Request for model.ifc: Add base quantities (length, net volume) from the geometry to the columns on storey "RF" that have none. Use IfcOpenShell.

First a look at what the model holds.

```python
import ifcopenshell
import ifcopenshell.util.element
import ifcopenshell.util.unit

model = ifcopenshell.open("model.ifc")
print(model.schema)
for unit_type in ("LENGTHUNIT", "AREAUNIT", "VOLUMEUNIT"):
    print(unit_type, ifcopenshell.util.unit.calculate_unit_scale(model, unit_type))
storey = next(s for s in model.by_type("IfcBuildingStorey") if s.Name == "RF")
columns = [e for e in ifcopenshell.util.element.get_decomposition(storey) if e.is_a("IfcColumn")]
for e in sorted(columns, key=lambda e: e.id()):
    print(e.id(), e.is_a(), e.Name, list(ifcopenshell.util.element.get_psets(e, qtos_only=True)), sep=" | ")
```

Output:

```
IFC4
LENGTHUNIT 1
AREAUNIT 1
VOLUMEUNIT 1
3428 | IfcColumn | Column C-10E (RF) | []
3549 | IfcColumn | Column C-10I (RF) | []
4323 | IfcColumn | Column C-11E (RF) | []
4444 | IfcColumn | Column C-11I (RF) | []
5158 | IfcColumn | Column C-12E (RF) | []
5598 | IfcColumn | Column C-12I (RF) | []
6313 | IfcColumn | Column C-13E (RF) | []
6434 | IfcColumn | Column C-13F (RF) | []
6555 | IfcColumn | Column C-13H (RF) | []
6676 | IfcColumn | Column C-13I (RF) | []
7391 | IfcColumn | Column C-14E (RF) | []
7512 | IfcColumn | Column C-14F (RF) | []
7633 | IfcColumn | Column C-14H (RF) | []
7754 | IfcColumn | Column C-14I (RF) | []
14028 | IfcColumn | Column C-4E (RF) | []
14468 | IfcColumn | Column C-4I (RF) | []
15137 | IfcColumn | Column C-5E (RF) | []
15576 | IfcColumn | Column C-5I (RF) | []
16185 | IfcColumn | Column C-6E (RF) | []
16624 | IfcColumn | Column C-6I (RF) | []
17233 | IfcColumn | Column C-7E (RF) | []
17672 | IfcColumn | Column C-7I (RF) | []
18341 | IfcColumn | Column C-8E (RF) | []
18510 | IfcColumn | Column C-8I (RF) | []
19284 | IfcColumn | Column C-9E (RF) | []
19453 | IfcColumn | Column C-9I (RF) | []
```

```python
import ifcopenshell
import ifcopenshell.api.pset
import ifcopenshell.geom
import ifcopenshell.util.element
import ifcopenshell.util.shape
import ifcopenshell.util.unit

model = ifcopenshell.open("model.ifc")
unit_scale = ifcopenshell.util.unit.calculate_unit_scale(model)
volume_scale = ifcopenshell.util.unit.calculate_unit_scale(model, "VOLUMEUNIT")
settings = ifcopenshell.geom.settings()

storey = next(s for s in model.by_type("IfcBuildingStorey") if s.Name == "RF")
columns = [e for e in ifcopenshell.util.element.get_decomposition(storey) if e.is_a("IfcColumn")]

for e in sorted(columns, key=lambda e: e.id()):
    if ifcopenshell.util.element.get_psets(e, qtos_only=True, should_inherit=False):
        continue
    # Geometry comes back in metres, in the element's own axes.
    shape = ifcopenshell.geom.create_shape(settings, e)
    values = {
        "Length": ifcopenshell.util.shape.get_z(shape.geometry) / unit_scale,
        "NetVolume": ifcopenshell.util.shape.get_volume(shape.geometry) / volume_scale,
    }
    qto = ifcopenshell.api.pset.add_qto(model, product=e, name="Qto_ColumnBaseQuantities")
    ifcopenshell.api.pset.edit_qto(model, qto=qto, properties=values)
    print(e.id(), {k: round(v, 3) for k, v in values.items()})

model.write("model_updated.ifc")
```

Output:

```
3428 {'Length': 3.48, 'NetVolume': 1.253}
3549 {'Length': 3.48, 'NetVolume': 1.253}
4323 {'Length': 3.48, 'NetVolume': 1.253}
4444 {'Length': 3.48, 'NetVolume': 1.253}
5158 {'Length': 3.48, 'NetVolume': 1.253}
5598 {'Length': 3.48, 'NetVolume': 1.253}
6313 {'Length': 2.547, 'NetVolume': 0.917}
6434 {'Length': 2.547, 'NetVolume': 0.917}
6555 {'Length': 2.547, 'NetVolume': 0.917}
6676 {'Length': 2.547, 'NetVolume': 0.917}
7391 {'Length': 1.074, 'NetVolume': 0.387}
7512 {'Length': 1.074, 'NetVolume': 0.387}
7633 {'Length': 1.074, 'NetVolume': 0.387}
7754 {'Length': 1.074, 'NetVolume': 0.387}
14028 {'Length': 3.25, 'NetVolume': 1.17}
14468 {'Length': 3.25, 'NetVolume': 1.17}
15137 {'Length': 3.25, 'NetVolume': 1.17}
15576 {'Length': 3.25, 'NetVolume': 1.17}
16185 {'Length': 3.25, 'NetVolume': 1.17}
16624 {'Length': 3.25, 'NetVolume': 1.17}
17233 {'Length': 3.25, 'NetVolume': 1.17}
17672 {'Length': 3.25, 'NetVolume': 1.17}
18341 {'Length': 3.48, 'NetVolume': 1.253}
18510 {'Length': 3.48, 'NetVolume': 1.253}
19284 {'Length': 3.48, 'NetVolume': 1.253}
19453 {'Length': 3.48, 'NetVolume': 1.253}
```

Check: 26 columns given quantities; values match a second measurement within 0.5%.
